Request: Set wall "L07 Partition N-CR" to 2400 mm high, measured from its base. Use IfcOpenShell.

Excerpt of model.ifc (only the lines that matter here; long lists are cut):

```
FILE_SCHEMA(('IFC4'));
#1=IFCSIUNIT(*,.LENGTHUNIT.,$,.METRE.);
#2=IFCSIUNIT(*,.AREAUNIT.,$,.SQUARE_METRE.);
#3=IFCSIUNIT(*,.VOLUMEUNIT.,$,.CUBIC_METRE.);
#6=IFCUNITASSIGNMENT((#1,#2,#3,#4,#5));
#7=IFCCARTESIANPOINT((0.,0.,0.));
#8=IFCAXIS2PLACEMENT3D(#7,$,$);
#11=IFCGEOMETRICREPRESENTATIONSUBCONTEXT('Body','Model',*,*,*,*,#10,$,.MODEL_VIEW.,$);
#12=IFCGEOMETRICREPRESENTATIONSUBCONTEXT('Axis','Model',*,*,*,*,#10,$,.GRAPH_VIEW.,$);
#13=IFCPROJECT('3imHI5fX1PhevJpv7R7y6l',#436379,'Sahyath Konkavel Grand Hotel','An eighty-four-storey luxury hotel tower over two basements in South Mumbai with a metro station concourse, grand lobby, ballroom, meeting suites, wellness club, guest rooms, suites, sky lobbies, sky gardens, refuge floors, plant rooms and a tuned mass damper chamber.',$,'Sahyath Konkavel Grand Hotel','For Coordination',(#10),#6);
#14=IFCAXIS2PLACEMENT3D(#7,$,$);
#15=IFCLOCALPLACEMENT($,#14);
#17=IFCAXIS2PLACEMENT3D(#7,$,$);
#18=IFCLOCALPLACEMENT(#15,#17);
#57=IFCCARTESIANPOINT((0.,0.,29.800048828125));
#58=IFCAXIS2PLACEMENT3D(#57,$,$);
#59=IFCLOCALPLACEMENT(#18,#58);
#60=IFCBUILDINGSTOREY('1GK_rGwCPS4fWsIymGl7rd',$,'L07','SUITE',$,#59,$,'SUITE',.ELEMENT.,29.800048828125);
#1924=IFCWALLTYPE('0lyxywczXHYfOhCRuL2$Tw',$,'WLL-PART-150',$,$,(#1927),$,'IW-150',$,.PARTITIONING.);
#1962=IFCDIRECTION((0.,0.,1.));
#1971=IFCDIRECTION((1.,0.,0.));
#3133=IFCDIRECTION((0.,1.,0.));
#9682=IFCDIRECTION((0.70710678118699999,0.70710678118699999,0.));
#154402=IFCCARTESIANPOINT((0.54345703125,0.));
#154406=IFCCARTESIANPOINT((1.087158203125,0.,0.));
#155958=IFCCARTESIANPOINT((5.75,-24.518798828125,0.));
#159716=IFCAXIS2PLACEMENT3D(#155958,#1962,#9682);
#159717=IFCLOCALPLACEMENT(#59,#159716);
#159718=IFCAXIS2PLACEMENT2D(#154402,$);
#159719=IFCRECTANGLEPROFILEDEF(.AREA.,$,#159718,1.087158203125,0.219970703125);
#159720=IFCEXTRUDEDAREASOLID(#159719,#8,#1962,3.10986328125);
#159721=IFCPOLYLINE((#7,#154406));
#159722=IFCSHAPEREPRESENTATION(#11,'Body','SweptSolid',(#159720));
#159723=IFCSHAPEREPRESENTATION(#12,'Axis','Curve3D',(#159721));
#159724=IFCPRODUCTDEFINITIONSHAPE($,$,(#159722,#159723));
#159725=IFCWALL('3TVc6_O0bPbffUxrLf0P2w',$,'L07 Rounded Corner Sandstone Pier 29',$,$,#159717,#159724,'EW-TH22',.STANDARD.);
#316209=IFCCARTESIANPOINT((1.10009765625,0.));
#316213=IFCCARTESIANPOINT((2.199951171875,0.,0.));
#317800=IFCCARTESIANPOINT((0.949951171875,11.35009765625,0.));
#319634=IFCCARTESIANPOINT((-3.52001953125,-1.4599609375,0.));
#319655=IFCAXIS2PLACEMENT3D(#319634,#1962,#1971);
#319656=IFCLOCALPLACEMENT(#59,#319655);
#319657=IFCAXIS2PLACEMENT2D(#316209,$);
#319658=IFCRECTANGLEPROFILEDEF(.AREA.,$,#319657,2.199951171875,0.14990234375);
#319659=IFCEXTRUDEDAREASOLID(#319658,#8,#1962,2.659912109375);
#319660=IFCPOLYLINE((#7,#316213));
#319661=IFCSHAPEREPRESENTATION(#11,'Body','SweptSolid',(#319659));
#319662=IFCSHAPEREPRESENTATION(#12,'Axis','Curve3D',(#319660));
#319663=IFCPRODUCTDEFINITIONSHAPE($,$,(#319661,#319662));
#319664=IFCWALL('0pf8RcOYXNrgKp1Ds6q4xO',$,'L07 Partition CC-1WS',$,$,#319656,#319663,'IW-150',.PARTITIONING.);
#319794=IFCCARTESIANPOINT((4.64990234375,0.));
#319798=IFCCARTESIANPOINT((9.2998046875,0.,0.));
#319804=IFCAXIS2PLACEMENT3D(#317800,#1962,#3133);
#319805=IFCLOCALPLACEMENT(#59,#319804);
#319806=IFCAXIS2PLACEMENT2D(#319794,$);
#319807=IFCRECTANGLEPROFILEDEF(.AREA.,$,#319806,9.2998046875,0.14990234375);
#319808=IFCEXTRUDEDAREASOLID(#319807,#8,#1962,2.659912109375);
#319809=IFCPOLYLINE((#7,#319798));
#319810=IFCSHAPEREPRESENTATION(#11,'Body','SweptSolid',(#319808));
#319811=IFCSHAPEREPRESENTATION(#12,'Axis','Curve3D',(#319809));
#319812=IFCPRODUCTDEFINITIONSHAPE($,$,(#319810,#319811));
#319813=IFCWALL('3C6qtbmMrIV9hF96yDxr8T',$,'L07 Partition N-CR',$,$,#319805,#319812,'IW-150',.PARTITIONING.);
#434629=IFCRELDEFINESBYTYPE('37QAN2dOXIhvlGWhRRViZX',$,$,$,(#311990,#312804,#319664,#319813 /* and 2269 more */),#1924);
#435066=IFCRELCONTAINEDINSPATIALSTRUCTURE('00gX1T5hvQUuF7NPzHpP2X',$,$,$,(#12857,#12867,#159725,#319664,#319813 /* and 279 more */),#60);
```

```python
import ifcopenshell
import ifcopenshell.geom
import ifcopenshell.util.representation
import ifcopenshell.util.shape
import ifcopenshell.util.unit

model = ifcopenshell.open("model.ifc")
unit_scale = ifcopenshell.util.unit.calculate_unit_scale(model)
settings = ifcopenshell.geom.settings()


def volume(element):
    """Net volume in cubic metres, openings subtracted."""
    shape = ifcopenshell.geom.create_shape(settings, element)
    return ifcopenshell.util.shape.get_volume(shape.geometry)


wall = model.by_guid("3C6qtbmMrIV9hF96yDxr8T")
before = volume(wall)

body = ifcopenshell.util.representation.get_representation(wall, "Model", "Body")
solid = body.Items[0]
old_height = solid.Depth
solid.Depth = 2.4 / unit_scale
after = volume(wall)

print(f"height {old_height:g} -> {solid.Depth:g}, volume {before:.3f} -> {after:.3f} m3")

model.write("model_rev.ifc")
```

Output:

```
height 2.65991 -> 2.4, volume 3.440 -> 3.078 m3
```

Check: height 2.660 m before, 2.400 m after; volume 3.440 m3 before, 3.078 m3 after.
